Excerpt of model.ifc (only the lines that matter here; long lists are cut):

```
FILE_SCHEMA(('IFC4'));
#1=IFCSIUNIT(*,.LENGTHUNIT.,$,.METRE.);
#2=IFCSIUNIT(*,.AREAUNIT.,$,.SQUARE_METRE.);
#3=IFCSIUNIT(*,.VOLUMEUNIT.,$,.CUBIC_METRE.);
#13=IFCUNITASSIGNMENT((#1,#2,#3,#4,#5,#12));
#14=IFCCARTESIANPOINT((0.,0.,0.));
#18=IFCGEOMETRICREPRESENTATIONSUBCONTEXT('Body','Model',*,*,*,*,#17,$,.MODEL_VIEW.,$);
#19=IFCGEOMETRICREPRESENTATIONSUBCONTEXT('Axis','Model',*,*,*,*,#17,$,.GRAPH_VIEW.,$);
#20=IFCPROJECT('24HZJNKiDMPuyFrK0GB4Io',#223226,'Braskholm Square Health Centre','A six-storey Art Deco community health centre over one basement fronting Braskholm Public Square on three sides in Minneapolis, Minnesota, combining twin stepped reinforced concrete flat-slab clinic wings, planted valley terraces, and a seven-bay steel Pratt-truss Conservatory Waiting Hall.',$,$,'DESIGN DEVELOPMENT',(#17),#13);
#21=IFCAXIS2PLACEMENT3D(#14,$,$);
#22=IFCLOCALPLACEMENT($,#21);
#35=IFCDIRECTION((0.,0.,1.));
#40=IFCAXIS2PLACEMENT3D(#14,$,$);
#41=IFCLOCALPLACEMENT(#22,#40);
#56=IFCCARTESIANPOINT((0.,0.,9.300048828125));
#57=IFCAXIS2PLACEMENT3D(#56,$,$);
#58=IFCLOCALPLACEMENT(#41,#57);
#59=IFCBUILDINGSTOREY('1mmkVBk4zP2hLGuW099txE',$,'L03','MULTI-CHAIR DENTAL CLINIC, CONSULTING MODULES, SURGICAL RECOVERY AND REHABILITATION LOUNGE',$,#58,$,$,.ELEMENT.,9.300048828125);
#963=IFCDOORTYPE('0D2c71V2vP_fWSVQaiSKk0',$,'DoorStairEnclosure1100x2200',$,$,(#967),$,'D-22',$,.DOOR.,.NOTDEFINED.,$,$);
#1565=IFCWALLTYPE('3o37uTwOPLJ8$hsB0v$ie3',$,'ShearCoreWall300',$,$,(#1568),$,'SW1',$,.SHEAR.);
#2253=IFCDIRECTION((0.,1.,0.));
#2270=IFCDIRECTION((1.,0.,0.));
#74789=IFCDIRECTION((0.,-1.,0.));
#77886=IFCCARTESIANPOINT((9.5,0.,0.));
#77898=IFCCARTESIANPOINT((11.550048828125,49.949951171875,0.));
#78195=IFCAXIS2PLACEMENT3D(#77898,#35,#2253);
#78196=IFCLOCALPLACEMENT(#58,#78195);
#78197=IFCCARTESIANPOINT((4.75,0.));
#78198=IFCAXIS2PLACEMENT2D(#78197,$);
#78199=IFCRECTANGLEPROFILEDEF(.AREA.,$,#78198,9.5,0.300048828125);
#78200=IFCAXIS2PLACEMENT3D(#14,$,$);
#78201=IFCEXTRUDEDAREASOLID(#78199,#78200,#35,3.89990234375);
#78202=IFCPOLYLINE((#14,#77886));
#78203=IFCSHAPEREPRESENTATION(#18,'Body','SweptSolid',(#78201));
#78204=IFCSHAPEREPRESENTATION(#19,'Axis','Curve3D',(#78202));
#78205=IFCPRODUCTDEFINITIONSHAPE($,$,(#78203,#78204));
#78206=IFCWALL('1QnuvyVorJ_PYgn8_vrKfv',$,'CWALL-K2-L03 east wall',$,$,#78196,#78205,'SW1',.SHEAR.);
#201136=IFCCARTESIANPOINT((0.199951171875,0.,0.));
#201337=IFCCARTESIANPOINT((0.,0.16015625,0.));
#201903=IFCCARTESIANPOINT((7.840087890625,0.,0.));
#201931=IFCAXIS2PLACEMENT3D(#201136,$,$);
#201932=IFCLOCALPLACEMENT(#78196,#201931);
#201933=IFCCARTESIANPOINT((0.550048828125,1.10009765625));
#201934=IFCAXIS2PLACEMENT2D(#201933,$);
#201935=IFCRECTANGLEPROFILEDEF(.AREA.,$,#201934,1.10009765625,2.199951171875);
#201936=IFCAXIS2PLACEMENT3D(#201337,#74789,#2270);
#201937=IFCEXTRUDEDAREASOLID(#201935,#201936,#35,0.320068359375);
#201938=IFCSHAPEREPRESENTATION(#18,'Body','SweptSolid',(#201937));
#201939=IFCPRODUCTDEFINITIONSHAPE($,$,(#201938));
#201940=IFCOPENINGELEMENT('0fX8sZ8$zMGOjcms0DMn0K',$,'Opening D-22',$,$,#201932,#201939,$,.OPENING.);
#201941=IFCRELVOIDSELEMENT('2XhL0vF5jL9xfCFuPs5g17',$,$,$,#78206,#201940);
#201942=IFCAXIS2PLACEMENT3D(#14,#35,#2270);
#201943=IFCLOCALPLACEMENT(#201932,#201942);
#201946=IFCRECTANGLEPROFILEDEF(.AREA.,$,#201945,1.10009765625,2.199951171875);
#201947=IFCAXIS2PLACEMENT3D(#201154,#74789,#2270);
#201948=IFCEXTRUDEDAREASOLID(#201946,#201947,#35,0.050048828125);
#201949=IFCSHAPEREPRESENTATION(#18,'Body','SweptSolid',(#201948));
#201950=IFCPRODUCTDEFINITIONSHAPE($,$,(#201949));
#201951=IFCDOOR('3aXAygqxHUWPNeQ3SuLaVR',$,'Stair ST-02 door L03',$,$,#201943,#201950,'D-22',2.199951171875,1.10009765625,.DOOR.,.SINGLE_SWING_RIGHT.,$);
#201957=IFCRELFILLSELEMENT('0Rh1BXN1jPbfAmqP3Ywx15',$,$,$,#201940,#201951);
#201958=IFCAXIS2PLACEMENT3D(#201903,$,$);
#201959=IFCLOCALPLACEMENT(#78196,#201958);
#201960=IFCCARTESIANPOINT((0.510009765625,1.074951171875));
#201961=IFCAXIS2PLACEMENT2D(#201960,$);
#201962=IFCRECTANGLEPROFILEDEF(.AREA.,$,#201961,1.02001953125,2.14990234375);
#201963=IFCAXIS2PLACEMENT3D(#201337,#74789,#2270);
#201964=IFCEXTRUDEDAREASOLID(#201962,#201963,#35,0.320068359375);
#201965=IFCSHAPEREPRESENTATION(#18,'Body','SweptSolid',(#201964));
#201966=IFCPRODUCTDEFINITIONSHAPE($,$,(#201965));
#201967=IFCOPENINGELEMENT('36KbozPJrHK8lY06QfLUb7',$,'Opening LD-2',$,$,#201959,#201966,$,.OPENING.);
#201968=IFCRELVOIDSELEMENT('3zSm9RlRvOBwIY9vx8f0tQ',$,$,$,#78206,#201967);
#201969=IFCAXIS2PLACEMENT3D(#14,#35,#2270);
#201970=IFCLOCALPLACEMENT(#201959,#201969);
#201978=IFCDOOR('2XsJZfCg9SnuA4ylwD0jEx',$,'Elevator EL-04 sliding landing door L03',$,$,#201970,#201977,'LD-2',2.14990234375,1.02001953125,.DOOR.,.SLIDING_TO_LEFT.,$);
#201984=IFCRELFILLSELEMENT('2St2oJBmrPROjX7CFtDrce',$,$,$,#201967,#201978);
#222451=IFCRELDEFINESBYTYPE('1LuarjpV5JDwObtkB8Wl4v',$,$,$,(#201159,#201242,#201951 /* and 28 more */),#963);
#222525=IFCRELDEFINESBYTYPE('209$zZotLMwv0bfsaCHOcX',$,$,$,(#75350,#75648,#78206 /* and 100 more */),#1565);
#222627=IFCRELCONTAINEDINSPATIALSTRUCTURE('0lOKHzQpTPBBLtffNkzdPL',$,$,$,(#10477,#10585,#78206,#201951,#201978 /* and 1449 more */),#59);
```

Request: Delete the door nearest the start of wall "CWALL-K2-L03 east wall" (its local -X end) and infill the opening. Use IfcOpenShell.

```python
import ifcopenshell
import ifcopenshell.api.feature
import ifcopenshell.api.root
import ifcopenshell.geom
import ifcopenshell.util.shape

model = ifcopenshell.open("model.ifc")
settings = ifcopenshell.geom.settings()


def volume(element):
    """Net volume in cubic metres, openings subtracted."""
    shape = ifcopenshell.geom.create_shape(settings, element)
    return ifcopenshell.util.shape.get_volume(shape.geometry)


door = model.by_guid("3aXAygqxHUWPNeQ3SuLaVR")
opening = door.FillsVoids[0].RelatingOpeningElement
wall = opening.VoidsElements[0].RelatingBuildingElement
before = volume(wall)

ifcopenshell.api.root.remove_product(model, product=door)
ifcopenshell.api.feature.remove_feature(model, feature=opening)

after = volume(wall)

print(f"wall volume {before:.3f} -> {after:.3f} m3")

model.write("model-out.ifc")
```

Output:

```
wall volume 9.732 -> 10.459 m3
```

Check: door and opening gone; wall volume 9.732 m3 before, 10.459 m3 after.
